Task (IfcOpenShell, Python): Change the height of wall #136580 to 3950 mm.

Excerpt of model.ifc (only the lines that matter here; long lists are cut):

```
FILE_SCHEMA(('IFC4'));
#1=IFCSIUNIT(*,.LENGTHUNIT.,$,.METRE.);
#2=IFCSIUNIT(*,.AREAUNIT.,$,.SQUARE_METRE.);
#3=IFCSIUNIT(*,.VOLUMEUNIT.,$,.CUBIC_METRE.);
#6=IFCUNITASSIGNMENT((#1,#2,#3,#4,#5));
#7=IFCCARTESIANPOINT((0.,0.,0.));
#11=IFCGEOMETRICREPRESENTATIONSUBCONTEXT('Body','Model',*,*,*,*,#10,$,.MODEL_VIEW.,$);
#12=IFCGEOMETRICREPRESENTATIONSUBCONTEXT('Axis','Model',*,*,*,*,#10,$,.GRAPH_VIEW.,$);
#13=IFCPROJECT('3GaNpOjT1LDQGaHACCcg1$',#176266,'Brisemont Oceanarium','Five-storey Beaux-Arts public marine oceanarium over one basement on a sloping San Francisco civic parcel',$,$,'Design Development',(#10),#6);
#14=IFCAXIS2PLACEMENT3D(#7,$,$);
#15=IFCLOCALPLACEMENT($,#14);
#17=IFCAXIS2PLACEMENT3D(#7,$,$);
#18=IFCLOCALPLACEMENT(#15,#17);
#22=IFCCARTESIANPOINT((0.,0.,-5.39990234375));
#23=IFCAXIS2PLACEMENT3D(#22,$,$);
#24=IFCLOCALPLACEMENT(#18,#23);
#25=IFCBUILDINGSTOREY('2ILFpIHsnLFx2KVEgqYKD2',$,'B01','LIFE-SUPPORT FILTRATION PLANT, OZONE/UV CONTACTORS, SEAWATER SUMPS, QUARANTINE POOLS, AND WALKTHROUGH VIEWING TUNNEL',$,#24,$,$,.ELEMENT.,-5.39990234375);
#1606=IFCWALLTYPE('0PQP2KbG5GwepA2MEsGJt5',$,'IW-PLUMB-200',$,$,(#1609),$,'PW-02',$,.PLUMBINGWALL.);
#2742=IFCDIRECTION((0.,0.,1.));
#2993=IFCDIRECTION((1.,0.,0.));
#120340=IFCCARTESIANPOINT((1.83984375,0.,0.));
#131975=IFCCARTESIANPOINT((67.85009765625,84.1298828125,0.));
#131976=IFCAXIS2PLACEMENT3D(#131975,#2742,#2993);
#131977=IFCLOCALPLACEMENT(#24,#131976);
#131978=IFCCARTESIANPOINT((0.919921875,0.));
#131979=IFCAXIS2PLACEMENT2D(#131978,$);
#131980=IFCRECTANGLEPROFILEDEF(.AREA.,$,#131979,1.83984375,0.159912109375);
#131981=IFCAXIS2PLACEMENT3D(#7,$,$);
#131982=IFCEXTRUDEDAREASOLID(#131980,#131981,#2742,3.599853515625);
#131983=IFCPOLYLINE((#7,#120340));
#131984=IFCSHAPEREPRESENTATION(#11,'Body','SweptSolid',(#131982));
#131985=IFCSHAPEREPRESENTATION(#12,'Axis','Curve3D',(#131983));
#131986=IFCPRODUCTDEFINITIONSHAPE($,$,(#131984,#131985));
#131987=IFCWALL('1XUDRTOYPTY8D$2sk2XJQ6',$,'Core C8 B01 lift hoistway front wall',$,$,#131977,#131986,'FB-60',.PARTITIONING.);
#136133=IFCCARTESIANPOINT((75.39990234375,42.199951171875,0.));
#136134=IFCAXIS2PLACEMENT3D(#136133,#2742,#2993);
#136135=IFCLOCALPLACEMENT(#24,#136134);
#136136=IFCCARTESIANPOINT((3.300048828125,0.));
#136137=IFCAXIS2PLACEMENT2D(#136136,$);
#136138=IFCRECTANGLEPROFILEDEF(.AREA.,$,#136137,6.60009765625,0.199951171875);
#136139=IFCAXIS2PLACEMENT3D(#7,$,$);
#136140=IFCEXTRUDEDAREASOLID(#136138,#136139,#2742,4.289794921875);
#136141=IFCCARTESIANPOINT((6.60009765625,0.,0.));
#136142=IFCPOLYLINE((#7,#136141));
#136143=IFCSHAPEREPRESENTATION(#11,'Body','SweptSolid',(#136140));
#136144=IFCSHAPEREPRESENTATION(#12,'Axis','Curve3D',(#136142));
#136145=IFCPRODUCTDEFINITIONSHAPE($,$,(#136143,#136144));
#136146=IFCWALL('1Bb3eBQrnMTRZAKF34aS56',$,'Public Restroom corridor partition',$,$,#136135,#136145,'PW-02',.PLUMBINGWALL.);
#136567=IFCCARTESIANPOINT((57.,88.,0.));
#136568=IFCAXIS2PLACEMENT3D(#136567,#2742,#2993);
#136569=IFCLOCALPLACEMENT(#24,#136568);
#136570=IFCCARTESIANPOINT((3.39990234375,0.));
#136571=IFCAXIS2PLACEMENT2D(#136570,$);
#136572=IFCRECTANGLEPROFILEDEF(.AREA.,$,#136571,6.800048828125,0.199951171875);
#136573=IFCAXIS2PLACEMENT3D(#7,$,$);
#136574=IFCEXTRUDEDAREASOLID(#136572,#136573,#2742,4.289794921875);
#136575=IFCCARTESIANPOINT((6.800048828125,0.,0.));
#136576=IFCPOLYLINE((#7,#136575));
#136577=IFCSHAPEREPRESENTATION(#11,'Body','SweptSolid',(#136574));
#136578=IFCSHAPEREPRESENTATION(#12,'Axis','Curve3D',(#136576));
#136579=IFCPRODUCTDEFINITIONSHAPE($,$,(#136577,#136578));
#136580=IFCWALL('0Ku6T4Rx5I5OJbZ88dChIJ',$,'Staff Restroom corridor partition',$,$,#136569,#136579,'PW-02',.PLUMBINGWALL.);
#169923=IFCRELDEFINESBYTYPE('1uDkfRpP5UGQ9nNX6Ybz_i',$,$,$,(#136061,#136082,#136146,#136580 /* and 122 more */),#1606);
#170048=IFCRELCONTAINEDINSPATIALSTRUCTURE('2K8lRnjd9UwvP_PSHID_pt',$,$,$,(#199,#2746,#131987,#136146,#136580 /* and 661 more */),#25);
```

```python
import ifcopenshell
import ifcopenshell.geom
import ifcopenshell.util.representation
import ifcopenshell.util.shape

model = ifcopenshell.open("model.ifc")
settings = ifcopenshell.geom.settings()


def volume(element):
    """Net volume in cubic metres, openings subtracted."""
    shape = ifcopenshell.geom.create_shape(settings, element)
    return ifcopenshell.util.shape.get_volume(shape.geometry)


wall = model.by_guid("0Ku6T4Rx5I5OJbZ88dChIJ")
before = volume(wall)

body = ifcopenshell.util.representation.get_representation(wall, "Model", "Body")
solid = body.Items[0]
old_height = solid.Depth
solid.Depth = 3.95
after = volume(wall)

print(f"height {old_height:g} -> {solid.Depth:g}, volume {before:.3f} -> {after:.3f} m3")

model.write("model-out.ifc")
```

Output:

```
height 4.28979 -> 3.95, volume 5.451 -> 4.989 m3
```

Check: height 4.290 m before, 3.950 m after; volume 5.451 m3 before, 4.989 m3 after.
